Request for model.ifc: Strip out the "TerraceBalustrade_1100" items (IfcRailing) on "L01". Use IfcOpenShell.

First a look at what the model holds.

```python
import ifcopenshell
import ifcopenshell.util.element

model = ifcopenshell.open("model.ifc")
print(model.schema)
storey = next(s for s in model.by_type("IfcBuildingStorey") if s.Name == "L01")
railings = [e for e in ifcopenshell.util.element.get_decomposition(storey) if e.is_a("IfcRailing")]
seen = {}
for e in railings:
    element_type = ifcopenshell.util.element.get_type(e)
    name = element_type.Name if element_type not in (None, e) else None
    seen[name] = seen.get(name, 0) + 1
for name, count in sorted(seen.items(), key=str):
    print(count, "x", name)
```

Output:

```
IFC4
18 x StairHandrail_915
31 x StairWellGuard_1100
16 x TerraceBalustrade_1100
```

```python
import ifcopenshell
import ifcopenshell.api.root
import ifcopenshell.util.element

model = ifcopenshell.open("model.ifc")

storey = next(s for s in model.by_type("IfcBuildingStorey") if s.Name == "L01")
railings = [e for e in ifcopenshell.util.element.get_decomposition(storey) if e.is_a("IfcRailing")]
targets = [e for e in railings if (t := ifcopenshell.util.element.get_type(e)) not in (None, e) and t.Name == "TerraceBalustrade_1100"]

for e in targets:
    ifcopenshell.api.root.remove_product(model, product=e)
print(len(targets), "removed")

model.write("model-out.ifc")
```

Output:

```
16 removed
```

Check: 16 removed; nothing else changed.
